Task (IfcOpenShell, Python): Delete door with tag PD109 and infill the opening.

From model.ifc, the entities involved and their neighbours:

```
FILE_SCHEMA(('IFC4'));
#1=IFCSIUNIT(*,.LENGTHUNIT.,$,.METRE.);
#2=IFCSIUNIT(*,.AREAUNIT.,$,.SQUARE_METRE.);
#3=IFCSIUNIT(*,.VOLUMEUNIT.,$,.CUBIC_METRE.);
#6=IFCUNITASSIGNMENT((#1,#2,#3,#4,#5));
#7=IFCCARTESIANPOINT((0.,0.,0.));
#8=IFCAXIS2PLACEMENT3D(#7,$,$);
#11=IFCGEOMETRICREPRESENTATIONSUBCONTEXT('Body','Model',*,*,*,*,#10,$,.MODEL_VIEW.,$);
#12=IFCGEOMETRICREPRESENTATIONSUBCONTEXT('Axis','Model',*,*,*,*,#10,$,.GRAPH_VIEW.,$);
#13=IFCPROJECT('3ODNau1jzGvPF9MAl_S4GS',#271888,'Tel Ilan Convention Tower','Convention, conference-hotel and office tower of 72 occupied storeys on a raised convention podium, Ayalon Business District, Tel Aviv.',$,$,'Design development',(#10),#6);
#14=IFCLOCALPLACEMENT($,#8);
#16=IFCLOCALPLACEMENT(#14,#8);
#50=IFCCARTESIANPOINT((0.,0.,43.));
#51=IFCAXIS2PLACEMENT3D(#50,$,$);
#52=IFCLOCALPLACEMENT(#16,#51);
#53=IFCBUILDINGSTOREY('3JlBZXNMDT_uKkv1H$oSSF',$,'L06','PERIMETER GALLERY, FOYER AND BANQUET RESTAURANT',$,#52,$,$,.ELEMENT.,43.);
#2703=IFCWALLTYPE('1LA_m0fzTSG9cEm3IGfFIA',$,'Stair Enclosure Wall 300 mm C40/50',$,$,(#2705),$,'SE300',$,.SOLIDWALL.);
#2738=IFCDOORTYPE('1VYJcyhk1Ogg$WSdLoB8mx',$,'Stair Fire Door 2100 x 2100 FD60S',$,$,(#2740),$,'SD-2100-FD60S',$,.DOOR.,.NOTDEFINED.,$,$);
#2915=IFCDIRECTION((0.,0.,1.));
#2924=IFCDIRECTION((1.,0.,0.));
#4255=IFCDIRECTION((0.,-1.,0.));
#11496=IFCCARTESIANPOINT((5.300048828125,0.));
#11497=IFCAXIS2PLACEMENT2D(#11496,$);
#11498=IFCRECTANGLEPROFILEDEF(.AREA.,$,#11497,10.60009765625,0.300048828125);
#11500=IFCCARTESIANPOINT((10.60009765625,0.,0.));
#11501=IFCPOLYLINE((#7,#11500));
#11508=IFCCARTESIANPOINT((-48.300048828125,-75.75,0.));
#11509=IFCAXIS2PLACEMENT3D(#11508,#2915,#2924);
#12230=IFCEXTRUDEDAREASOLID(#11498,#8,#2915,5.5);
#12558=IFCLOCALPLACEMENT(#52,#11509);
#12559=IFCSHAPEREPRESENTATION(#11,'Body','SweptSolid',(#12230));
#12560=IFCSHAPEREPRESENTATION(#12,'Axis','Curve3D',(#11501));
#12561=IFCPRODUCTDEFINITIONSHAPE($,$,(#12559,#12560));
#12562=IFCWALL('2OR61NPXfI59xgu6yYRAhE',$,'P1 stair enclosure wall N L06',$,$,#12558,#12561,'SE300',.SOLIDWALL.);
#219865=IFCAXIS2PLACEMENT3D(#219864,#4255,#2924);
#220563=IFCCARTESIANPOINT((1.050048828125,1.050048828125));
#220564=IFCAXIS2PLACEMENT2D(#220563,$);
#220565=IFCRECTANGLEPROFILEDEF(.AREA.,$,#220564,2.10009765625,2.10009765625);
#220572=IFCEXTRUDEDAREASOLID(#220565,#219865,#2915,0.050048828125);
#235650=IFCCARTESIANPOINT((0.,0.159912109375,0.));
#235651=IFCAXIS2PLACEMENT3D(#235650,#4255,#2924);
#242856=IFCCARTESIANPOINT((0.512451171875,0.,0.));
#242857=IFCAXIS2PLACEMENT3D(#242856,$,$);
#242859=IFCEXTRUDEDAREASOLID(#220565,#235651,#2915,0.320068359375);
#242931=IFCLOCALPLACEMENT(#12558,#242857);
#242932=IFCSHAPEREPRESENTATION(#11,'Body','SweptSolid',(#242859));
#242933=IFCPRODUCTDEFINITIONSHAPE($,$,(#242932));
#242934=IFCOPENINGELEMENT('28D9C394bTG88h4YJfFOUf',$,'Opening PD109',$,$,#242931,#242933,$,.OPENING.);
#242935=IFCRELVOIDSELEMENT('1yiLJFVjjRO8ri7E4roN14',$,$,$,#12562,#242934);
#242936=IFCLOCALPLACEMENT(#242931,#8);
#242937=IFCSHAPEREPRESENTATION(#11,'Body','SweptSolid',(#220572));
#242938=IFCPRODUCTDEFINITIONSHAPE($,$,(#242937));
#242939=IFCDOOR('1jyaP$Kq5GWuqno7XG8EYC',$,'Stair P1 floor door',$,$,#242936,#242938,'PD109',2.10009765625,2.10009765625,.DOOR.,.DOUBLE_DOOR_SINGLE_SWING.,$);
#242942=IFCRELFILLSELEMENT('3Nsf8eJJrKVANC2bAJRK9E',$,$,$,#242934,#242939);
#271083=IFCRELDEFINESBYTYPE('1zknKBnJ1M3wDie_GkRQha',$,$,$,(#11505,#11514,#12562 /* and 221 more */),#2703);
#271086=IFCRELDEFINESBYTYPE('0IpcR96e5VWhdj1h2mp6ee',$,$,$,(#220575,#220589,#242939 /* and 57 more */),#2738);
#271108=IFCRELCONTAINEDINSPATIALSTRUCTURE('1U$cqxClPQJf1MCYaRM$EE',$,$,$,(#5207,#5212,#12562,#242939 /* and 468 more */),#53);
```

```python
import ifcopenshell
import ifcopenshell.api.feature
import ifcopenshell.api.root
import ifcopenshell.geom
import ifcopenshell.util.shape

model = ifcopenshell.open("model.ifc")
settings = ifcopenshell.geom.settings()


def volume(element):
    """Net volume in cubic metres, openings subtracted."""
    shape = ifcopenshell.geom.create_shape(settings, element)
    return ifcopenshell.util.shape.get_volume(shape.geometry)


door = model.by_guid("1jyaP$Kq5GWuqno7XG8EYC")
opening = door.FillsVoids[0].RelatingOpeningElement
wall = opening.VoidsElements[0].RelatingBuildingElement
before = volume(wall)

ifcopenshell.api.root.remove_product(model, product=door)
ifcopenshell.api.feature.remove_feature(model, feature=opening)

after = volume(wall)

print(f"wall volume {before:.3f} -> {after:.3f} m3")

model.write("model_edited.ifc")
```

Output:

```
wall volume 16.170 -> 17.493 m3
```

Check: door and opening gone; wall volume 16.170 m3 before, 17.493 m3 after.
